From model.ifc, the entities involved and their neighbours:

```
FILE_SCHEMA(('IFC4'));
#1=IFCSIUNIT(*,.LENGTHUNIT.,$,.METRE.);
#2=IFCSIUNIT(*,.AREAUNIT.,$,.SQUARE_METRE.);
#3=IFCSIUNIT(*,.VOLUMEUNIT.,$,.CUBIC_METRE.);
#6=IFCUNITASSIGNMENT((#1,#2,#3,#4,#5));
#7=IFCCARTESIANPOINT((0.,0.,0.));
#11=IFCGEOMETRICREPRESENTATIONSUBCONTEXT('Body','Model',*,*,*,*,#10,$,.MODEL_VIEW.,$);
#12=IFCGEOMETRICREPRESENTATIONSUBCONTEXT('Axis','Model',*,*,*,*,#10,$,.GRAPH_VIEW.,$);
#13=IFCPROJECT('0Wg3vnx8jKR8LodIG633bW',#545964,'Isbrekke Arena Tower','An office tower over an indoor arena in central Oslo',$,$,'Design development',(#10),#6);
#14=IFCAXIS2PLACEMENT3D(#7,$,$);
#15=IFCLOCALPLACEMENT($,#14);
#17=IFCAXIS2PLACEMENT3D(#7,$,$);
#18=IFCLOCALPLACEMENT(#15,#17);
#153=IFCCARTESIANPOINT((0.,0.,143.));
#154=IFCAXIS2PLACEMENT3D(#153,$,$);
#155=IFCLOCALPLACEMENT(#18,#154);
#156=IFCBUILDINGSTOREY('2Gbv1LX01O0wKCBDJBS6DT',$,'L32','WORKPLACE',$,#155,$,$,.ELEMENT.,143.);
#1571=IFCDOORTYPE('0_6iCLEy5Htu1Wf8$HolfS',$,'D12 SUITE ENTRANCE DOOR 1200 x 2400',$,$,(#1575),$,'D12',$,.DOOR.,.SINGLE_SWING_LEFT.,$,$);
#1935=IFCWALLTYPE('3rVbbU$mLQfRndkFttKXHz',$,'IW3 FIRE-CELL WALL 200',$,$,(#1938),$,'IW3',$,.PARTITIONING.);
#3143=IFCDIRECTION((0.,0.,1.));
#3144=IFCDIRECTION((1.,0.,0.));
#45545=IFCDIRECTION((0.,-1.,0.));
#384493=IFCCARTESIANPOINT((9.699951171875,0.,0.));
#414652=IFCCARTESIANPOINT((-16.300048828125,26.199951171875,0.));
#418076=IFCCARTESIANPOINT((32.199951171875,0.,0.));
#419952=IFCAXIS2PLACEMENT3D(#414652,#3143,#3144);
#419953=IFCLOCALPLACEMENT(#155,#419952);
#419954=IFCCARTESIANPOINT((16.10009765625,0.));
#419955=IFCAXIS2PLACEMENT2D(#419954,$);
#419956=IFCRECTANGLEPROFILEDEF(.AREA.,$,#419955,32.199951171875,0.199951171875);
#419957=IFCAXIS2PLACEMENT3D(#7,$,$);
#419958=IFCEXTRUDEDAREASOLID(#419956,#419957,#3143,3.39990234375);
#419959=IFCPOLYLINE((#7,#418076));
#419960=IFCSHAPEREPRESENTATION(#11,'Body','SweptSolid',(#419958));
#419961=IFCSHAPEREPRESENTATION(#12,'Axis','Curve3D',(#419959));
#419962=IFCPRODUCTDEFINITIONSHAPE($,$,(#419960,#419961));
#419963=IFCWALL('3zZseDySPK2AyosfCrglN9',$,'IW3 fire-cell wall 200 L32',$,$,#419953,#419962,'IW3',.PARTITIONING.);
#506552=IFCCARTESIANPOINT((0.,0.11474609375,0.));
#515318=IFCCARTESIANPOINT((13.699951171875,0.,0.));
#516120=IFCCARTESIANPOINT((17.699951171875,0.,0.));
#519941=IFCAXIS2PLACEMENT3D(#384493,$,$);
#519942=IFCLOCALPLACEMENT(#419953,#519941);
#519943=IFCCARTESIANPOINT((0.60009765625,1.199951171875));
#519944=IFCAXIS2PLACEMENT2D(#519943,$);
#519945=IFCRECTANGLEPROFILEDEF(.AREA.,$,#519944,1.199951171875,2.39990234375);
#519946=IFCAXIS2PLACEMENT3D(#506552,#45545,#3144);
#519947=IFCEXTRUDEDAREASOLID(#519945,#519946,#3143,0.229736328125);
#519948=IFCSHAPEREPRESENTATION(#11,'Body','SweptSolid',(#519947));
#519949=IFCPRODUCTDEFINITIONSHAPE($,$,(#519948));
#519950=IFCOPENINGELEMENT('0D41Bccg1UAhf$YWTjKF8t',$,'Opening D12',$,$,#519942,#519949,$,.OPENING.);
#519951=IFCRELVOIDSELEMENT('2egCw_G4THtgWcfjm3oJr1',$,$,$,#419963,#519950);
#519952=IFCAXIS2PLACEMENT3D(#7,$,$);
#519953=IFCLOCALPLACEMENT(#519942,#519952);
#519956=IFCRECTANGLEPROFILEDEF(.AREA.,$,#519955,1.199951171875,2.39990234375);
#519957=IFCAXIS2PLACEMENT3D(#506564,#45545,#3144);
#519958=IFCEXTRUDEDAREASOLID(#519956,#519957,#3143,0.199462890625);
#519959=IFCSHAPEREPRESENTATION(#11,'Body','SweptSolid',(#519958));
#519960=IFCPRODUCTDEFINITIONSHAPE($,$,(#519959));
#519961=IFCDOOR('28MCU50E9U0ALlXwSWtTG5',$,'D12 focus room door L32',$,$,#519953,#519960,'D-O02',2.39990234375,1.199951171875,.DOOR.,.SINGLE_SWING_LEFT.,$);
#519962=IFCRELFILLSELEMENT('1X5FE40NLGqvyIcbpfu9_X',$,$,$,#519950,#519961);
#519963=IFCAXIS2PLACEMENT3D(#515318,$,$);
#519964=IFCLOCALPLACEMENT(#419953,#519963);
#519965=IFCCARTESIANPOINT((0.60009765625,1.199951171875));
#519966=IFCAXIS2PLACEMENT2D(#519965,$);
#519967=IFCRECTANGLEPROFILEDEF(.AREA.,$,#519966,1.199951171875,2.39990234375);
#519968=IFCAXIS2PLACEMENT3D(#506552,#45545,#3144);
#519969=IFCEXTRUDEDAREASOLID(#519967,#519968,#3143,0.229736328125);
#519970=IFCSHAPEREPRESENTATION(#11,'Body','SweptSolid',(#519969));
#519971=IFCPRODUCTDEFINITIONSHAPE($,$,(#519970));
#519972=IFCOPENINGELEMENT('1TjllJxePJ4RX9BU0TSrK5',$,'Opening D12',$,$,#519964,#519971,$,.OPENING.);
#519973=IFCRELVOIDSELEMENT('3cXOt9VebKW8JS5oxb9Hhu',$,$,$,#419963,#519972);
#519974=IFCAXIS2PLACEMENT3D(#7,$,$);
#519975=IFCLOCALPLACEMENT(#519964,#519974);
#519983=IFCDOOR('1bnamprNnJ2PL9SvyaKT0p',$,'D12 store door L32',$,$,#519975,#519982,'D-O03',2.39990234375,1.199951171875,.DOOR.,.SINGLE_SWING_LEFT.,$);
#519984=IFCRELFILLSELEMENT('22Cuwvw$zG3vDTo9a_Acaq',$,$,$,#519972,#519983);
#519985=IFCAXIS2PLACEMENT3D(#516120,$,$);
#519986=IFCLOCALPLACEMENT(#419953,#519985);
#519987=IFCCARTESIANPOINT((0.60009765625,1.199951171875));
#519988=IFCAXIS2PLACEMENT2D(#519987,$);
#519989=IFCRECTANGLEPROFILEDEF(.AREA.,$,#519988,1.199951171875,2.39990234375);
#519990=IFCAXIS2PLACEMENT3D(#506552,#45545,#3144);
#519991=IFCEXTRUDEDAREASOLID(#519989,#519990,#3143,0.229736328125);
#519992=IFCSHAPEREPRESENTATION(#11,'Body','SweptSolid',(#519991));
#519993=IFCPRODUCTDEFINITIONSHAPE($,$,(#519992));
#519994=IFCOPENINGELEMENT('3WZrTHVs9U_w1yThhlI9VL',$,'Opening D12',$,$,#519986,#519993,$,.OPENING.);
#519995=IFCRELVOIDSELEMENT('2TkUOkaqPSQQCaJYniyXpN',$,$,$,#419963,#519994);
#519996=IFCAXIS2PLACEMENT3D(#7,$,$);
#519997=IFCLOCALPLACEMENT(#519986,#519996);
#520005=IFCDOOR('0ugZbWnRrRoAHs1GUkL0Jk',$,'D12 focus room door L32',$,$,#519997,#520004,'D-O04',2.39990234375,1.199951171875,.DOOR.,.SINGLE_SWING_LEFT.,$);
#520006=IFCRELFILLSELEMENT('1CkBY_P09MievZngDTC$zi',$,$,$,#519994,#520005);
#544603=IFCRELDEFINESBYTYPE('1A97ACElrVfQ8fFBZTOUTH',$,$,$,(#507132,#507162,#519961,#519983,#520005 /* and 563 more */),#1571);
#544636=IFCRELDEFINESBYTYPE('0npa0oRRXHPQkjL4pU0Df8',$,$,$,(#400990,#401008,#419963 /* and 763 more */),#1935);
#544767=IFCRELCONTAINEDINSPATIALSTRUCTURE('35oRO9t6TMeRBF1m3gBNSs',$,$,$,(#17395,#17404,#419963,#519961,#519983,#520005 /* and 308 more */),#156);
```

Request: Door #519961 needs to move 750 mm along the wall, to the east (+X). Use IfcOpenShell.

```python
import ifcopenshell
import ifcopenshell.api.geometry
import ifcopenshell.util.placement
import ifcopenshell.util.unit

model = ifcopenshell.open("model.ifc")
unit_scale = ifcopenshell.util.unit.calculate_unit_scale(model)

door = model.by_guid("28MCU50E9U0ALlXwSWtTG5")
opening = door.FillsVoids[0].RelatingOpeningElement
wall = opening.VoidsElements[0].RelatingBuildingElement

wall_matrix = ifcopenshell.util.placement.get_local_placement(wall.ObjectPlacement)
shift = wall_matrix[:3, 0] * 0.75 / unit_scale
before = ifcopenshell.util.placement.get_local_placement(door.ObjectPlacement)[:3, 3].copy()

# The door is placed relative to its opening, so it follows when the opening moves.
matrix = ifcopenshell.util.placement.get_local_placement(opening.ObjectPlacement)
matrix[:3, 3] += shift
ifcopenshell.api.geometry.edit_object_placement(
    model, product=opening, matrix=matrix, is_si=False, should_transform_children=True
)

after = ifcopenshell.util.placement.get_local_placement(door.ObjectPlacement)[:3, 3]
print("door moved by", (after - before).round(3) + 0.0)

model.write("model-out.ifc")
```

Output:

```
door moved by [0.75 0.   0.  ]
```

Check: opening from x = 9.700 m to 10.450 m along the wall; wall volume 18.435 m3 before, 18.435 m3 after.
